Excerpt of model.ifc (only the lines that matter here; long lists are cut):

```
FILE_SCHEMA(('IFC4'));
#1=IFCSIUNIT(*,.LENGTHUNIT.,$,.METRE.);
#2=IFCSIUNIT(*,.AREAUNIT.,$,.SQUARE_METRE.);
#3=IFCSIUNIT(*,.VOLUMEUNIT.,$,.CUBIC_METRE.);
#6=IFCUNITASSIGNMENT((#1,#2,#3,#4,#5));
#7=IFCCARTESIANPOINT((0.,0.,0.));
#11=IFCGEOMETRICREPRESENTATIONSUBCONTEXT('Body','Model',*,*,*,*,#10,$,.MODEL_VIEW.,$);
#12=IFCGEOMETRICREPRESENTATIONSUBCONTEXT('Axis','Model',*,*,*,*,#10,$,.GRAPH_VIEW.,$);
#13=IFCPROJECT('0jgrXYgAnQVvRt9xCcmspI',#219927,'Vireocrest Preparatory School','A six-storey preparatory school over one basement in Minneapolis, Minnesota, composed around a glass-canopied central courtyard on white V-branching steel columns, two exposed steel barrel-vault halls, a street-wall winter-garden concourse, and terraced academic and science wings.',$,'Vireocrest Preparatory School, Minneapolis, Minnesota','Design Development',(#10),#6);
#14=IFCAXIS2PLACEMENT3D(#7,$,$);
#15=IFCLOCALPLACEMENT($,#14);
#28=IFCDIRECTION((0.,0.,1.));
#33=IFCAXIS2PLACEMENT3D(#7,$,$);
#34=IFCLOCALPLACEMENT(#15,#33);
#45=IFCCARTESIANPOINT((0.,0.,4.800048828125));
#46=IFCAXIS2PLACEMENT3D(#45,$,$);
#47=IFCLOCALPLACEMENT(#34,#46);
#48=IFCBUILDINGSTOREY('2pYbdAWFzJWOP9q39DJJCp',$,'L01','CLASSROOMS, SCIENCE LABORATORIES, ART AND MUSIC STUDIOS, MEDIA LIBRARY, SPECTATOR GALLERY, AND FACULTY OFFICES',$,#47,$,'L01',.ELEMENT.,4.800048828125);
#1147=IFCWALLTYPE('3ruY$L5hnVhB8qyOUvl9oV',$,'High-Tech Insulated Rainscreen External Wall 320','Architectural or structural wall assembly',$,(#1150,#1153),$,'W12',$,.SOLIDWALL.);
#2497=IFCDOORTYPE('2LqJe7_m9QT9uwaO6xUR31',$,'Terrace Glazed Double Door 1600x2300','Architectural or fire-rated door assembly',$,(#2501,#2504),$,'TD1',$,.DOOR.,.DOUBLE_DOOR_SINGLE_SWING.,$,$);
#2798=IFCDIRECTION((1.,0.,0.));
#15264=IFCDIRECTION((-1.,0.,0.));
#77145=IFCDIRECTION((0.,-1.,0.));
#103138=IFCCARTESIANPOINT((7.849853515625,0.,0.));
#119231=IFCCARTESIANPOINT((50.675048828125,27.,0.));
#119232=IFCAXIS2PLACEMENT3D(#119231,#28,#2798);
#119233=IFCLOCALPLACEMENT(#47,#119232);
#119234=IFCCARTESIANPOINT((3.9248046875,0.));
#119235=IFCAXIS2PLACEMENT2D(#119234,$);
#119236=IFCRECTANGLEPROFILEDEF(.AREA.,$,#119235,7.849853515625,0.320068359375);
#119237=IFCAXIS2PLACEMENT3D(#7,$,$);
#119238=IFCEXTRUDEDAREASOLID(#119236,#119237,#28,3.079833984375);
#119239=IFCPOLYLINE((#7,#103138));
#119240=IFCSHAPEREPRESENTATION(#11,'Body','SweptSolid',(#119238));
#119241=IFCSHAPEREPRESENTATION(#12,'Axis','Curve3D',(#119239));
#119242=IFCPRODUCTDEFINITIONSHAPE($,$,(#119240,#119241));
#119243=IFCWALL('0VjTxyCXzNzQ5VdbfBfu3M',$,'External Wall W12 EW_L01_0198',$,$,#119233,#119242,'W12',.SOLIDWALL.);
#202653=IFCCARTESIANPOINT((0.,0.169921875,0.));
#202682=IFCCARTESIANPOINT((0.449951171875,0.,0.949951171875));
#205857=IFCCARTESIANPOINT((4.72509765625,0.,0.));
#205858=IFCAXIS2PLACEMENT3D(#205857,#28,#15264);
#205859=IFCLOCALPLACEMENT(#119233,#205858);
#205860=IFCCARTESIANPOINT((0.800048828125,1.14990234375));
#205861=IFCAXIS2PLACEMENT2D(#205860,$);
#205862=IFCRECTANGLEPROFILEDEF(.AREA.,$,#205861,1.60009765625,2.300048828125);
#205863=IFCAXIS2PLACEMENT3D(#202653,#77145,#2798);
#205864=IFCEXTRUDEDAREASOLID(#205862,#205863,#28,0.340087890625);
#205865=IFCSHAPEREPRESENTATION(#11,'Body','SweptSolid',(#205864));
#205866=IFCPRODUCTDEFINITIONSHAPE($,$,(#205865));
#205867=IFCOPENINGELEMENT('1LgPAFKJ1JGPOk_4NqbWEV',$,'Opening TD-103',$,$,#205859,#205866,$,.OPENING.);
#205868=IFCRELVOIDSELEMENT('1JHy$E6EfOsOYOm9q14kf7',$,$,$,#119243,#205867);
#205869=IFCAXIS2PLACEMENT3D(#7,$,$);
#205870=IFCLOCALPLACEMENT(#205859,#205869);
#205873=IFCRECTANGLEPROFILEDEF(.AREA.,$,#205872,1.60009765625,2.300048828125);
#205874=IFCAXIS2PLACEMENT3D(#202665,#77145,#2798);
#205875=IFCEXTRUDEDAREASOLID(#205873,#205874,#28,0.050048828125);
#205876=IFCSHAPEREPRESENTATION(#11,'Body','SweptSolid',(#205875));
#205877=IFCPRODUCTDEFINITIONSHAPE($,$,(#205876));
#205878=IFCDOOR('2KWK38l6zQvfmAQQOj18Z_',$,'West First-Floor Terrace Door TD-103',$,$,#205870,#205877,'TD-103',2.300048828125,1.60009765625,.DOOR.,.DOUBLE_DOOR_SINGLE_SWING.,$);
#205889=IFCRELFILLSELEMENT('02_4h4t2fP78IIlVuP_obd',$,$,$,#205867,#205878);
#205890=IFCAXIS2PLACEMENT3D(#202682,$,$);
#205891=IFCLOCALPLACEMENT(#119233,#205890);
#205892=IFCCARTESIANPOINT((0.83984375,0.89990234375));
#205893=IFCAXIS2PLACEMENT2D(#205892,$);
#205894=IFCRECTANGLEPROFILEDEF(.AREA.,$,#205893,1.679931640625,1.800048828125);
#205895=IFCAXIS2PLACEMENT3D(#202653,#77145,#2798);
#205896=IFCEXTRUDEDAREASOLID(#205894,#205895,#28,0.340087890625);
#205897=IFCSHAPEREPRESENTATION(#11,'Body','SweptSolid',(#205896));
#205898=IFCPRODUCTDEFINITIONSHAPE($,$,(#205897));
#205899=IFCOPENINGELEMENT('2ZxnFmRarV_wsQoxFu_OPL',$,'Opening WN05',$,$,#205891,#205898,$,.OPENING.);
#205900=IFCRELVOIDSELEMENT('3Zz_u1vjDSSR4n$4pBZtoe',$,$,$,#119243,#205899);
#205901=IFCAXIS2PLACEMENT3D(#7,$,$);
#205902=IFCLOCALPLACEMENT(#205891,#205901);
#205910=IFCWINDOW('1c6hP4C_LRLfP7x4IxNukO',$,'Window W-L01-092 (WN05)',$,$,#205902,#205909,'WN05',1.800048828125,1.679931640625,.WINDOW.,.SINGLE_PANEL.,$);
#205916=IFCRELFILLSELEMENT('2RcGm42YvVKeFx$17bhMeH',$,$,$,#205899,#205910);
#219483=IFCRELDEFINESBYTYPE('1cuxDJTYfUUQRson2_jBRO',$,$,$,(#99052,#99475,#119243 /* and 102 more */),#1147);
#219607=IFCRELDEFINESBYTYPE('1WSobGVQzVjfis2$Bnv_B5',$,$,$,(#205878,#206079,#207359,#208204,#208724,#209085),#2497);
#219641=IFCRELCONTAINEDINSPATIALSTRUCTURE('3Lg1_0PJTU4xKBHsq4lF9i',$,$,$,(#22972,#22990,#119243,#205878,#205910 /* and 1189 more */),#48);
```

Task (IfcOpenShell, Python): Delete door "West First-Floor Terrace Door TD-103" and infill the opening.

```python
import ifcopenshell
import ifcopenshell.api.feature
import ifcopenshell.api.root
import ifcopenshell.geom
import ifcopenshell.util.shape

model = ifcopenshell.open("model.ifc")
settings = ifcopenshell.geom.settings()


def volume(element):
    """Net volume in cubic metres, openings subtracted."""
    shape = ifcopenshell.geom.create_shape(settings, element)
    return ifcopenshell.util.shape.get_volume(shape.geometry)


door = model.by_id(205878)
opening = door.FillsVoids[0].RelatingOpeningElement
wall = opening.VoidsElements[0].RelatingBuildingElement
before = volume(wall)

ifcopenshell.api.root.remove_product(model, product=door)
ifcopenshell.api.feature.remove_feature(model, feature=opening)

after = volume(wall)

print(f"wall volume {before:.3f} -> {after:.3f} m3")

model.write("model-out.ifc")
```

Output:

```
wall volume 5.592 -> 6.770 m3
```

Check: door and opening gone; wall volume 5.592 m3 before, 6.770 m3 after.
